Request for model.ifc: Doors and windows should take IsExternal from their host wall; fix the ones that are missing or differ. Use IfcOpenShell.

First a look at what the model holds.

```python
import ifcopenshell
import ifcopenshell.util.element

model = ifcopenshell.open("model.ifc")
print(model.schema)
seen = {}
for e in model.by_type("IfcDoor") + model.by_type("IfcWindow"):
    if not e.FillsVoids:
        continue
    host = e.FillsVoids[0].RelatingOpeningElement.VoidsElements[0].RelatingBuildingElement
    own = ifcopenshell.util.element.get_pset(e, f"Pset_{e.is_a()[3:].removesuffix('StandardCase')}Common", "IsExternal")
    wall = ifcopenshell.util.element.get_pset(host, "Pset_WallCommon", "IsExternal")
    seen[e.is_a(), own, wall] = seen.get((e.is_a(), own, wall), 0) + 1
for (cls, own, wall), count in sorted(seen.items(), key=str):
    print(count, cls, "IsExternal:", own, "| host wall:", wall)
```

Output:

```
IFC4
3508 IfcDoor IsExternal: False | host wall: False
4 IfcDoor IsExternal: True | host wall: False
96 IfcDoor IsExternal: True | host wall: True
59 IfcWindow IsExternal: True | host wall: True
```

```python
import ifcopenshell
import ifcopenshell.api.pset
import ifcopenshell.util.element

model = ifcopenshell.open("model.ifc")

count = 0
for ifc_class, pset_name in (("IfcDoor", "Pset_DoorCommon"), ("IfcWindow", "Pset_WindowCommon")):
    for e in model.by_type(ifc_class):
        if not e.FillsVoids:
            continue
        host = e.FillsVoids[0].RelatingOpeningElement.VoidsElements[0].RelatingBuildingElement
        external = ifcopenshell.util.element.get_pset(host, "Pset_WallCommon", "IsExternal")
        if external is None or ifcopenshell.util.element.get_pset(e, pset_name, "IsExternal") == external:
            continue
        pset = ifcopenshell.api.pset.add_pset(model, product=e, name=pset_name)
        ifcopenshell.api.pset.edit_pset(model, pset=pset, properties={"IsExternal": external})
        count += 1

print(count, "updated")

model.write("model_rev.ifc")
```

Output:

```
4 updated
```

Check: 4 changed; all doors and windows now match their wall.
